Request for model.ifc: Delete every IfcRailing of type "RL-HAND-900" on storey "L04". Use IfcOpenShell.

First a look at what the model holds.

```python
import ifcopenshell
import ifcopenshell.util.element

model = ifcopenshell.open("model.ifc")
print(model.schema)
storey = next(s for s in model.by_type("IfcBuildingStorey") if s.Name == "L04")
railings = [e for e in ifcopenshell.util.element.get_decomposition(storey) if e.is_a("IfcRailing")]
seen = {}
for e in railings:
    element_type = ifcopenshell.util.element.get_type(e)
    name = element_type.Name if element_type not in (None, e) else None
    seen[name] = seen.get(name, 0) + 1
for name, count in sorted(seen.items(), key=str):
    print(count, "x", name)
```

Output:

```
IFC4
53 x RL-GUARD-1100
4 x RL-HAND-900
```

```python
import ifcopenshell
import ifcopenshell.api.root
import ifcopenshell.util.element

model = ifcopenshell.open("model.ifc")

storey = next(s for s in model.by_type("IfcBuildingStorey") if s.Name == "L04")
railings = [e for e in ifcopenshell.util.element.get_decomposition(storey) if e.is_a("IfcRailing")]
targets = [e for e in railings if (t := ifcopenshell.util.element.get_type(e)) not in (None, e) and t.Name == "RL-HAND-900"]

for e in targets:
    ifcopenshell.api.root.remove_product(model, product=e)
print(len(targets), "removed")

model.write("model_rev.ifc")
```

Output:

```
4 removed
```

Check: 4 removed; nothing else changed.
